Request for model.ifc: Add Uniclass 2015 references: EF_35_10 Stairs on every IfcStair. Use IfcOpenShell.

First a look at what the model holds.

```python
import ifcopenshell

model = ifcopenshell.open("model.ifc")
print(model.schema)
print("classifications:", [c.Name for c in model.by_type("IfcClassification")])
for ifc_class in ("IfcDoor", "IfcRoof", "IfcStair", "IfcWall", "IfcWindow"):
    print(ifc_class, len(model.by_type(ifc_class)))
```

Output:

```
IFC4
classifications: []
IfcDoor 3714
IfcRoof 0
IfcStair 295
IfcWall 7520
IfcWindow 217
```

```python
import ifcopenshell
import ifcopenshell.api.classification

model = ifcopenshell.open("model.ifc")

system = ifcopenshell.api.classification.add_classification(model, classification="Uniclass 2015")

codes = {
    "IfcStair": ("EF_35_10", "Stairs"),
}
for ifc_class, (code, name) in codes.items():
    products = model.by_type(ifc_class)
    ifcopenshell.api.classification.add_reference(
        model, products=products, classification=system, identification=code, name=name
    )
    print(code, len(products))

model.write("model-out.ifc")
```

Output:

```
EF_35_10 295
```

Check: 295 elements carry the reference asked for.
